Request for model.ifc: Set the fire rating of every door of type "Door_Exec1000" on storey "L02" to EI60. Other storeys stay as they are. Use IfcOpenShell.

First a look at what the model holds.

```python
import ifcopenshell
import ifcopenshell.util.element

model = ifcopenshell.open("model.ifc")
print(model.schema)
storey = next(s for s in model.by_type("IfcBuildingStorey") if s.Name == "L02")
doors = [e for e in ifcopenshell.util.element.get_decomposition(storey) if e.is_a("IfcDoor")]
seen = {}
for e in doors:
    element_type = ifcopenshell.util.element.get_type(e)
    key = (element_type.Name if element_type != e and element_type else None, ifcopenshell.util.element.get_pset(e, "Pset_DoorCommon", "FireRating"))
    seen[key] = seen.get(key, 0) + 1
for (name, value), count in sorted(seen.items(), key=str):
    print(count, "x", name, "|", value)
```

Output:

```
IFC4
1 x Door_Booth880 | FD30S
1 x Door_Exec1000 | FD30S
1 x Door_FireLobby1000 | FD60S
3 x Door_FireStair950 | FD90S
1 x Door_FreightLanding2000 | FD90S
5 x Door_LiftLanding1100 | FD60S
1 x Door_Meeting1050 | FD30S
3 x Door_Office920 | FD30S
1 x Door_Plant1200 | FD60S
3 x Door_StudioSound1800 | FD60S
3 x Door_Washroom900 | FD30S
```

```python
import ifcopenshell
import ifcopenshell.api.pset
import ifcopenshell.util.element

model = ifcopenshell.open("model.ifc")

storey = next(s for s in model.by_type("IfcBuildingStorey") if s.Name == "L02")
doors = [e for e in ifcopenshell.util.element.get_decomposition(storey) if e.is_a("IfcDoor")]

count = 0
for e in doors:
    element_type = ifcopenshell.util.element.get_type(e)
    if element_type in (None, e) or element_type.Name != "Door_Exec1000":
        continue
    # add_pset returns the element's existing set when there is one.
    pset = ifcopenshell.api.pset.add_pset(model, product=e, name="Pset_DoorCommon")
    ifcopenshell.api.pset.edit_pset(model, pset=pset, properties={"FireRating": "EI60"})
    count += 1

print(count, "doors updated")

model.write("model-out.ifc")
```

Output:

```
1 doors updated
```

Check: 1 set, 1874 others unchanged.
